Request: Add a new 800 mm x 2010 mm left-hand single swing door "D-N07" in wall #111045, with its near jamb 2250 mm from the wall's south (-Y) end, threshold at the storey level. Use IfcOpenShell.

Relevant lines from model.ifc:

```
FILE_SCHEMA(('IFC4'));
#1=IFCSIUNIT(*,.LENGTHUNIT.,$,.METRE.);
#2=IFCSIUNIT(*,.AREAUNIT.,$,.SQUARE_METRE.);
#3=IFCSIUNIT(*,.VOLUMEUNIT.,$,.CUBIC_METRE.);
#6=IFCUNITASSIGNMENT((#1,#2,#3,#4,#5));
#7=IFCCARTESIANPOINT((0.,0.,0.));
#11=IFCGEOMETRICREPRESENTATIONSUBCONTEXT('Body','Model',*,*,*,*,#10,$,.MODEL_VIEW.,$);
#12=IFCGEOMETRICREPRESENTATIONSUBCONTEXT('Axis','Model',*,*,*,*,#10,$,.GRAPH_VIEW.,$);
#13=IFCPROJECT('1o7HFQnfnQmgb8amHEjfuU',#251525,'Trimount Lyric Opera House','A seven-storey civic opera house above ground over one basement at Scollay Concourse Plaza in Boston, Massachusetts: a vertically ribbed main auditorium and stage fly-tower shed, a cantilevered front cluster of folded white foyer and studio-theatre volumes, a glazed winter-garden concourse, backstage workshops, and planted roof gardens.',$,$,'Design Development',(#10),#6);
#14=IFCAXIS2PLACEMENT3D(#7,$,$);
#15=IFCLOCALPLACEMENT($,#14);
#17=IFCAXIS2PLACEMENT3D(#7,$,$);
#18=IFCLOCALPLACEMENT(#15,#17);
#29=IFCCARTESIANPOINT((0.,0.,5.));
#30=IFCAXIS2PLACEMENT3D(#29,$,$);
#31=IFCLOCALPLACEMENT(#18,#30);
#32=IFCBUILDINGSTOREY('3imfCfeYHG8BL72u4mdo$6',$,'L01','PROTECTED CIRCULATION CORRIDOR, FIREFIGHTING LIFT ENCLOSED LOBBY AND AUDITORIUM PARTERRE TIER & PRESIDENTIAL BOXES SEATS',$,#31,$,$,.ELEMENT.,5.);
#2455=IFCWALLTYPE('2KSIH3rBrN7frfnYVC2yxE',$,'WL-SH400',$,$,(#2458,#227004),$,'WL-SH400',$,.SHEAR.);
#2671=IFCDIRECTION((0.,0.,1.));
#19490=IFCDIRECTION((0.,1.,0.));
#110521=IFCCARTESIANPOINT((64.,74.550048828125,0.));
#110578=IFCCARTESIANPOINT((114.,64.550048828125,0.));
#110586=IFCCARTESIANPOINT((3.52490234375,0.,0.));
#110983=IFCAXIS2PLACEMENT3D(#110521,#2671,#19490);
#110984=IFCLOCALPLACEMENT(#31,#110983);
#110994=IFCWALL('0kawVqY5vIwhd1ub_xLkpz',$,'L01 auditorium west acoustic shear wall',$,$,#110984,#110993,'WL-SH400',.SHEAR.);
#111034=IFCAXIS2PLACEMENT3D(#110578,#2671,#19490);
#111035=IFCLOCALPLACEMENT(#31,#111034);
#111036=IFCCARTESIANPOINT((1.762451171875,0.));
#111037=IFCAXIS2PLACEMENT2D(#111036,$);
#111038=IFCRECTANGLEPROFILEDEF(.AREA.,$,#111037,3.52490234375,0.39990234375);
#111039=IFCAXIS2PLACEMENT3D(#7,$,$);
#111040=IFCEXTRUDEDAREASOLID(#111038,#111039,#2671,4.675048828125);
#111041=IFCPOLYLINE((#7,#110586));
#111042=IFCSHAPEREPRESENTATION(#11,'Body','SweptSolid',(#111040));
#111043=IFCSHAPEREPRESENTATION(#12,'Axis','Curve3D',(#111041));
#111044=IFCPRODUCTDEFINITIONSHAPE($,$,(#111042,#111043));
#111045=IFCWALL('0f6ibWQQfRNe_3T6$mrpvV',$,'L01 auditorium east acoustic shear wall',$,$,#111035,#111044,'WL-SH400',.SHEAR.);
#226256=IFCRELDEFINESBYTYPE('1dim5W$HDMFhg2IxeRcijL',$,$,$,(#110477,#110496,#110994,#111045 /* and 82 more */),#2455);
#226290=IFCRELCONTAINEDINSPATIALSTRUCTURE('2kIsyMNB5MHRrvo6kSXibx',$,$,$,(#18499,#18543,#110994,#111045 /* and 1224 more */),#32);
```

```python
import numpy as np
import ifcopenshell
import ifcopenshell.api.feature
import ifcopenshell.api.geometry
import ifcopenshell.api.root
import ifcopenshell.api.spatial
import ifcopenshell.geom
import ifcopenshell.util.element
import ifcopenshell.util.placement
import ifcopenshell.util.representation
import ifcopenshell.util.shape
import ifcopenshell.util.unit

model = ifcopenshell.open("model.ifc")
unit_scale = ifcopenshell.util.unit.calculate_unit_scale(model)
settings = ifcopenshell.geom.settings()


def volume(element):
    """Net volume in cubic metres, openings subtracted."""
    shape = ifcopenshell.geom.create_shape(settings, element)
    return ifcopenshell.util.shape.get_volume(shape.geometry)


wall = model.by_guid("0f6ibWQQfRNe_3T6$mrpvV")
storey = ifcopenshell.util.element.get_container(wall, ifc_class="IfcBuildingStorey")
context = ifcopenshell.util.representation.get_context(model, "Model", "Body", "MODEL_VIEW")
before = volume(wall)

width, height, from_end, sill = 0.8, 2.01, 2.25, 0.0  # metres

# The wall runs along its own X axis, and the end named is its -X end.
wall_shape = ifcopenshell.geom.create_shape(settings, wall)
x, y, z = ifcopenshell.util.shape.get_vertices(wall_shape.geometry).T
start = x.min() + from_end
face, thickness = float(y.min()), float(y.max() - y.min())
wall_matrix = ifcopenshell.util.placement.get_local_placement(wall.ObjectPlacement)
level = ifcopenshell.util.placement.get_local_placement(storey.ObjectPlacement)[2, 3]


def in_wall(x, y):
    """Placement at x, y metres in the wall's axes, at sill height."""
    matrix = wall_matrix.copy()
    matrix[:, 3] = wall_matrix @ np.array([x / unit_scale, y / unit_scale, 0.0, 1.0])
    matrix[2, 3] = level + sill / unit_scale
    return matrix


# Opening: a box that overshoots both wall faces by 50 mm.
opening = ifcopenshell.api.root.create_entity(model, ifc_class="IfcOpeningElement", predefined_type="OPENING")
box = ifcopenshell.api.geometry.add_wall_representation(
    model, context=context, length=width, height=height, thickness=thickness + 0.1
)
ifcopenshell.api.geometry.assign_representation(model, product=opening, representation=box)
ifcopenshell.api.geometry.edit_object_placement(model, product=opening, matrix=in_wall(start, face - 0.05), is_si=False)
ifcopenshell.api.feature.add_feature(model, feature=opening, element=wall)

door = ifcopenshell.api.root.create_entity(model, ifc_class="IfcDoor", name="D-N07", predefined_type="DOOR")
door.OverallWidth, door.OverallHeight = width / unit_scale, height / unit_scale
door.OperationType = "SINGLE_SWING_LEFT"
body = ifcopenshell.api.geometry.add_door_representation(
    model,
    context=context,
    overall_width=door.OverallWidth,
    overall_height=door.OverallHeight,
    operation_type="SINGLE_SWING_LEFT",
    lining_properties={"LiningDepth": thickness / unit_scale, "ThresholdDepth": thickness / unit_scale},
)
ifcopenshell.api.geometry.assign_representation(model, product=door, representation=body)
ifcopenshell.api.spatial.assign_container(model, products=[door], relating_structure=storey)
ifcopenshell.api.feature.add_filling(model, opening=opening, element=door)

# The lining spans the wall, so the door starts at the wall face.
ifcopenshell.api.geometry.edit_object_placement(model, product=door, matrix=in_wall(start, face), is_si=False)

after = volume(wall)

print(f"wall volume {before:.3f} -> {after:.3f} m3")

model.write("model-out.ifc")
```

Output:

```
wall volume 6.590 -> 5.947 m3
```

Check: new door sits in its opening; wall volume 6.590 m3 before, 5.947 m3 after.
